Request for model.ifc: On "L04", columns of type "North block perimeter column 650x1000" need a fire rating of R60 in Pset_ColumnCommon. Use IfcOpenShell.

First a look at what the model holds.

```python
import ifcopenshell
import ifcopenshell.util.element

model = ifcopenshell.open("model.ifc")
print(model.schema)
storey = next(s for s in model.by_type("IfcBuildingStorey") if s.Name == "L04")
columns = [e for e in ifcopenshell.util.element.get_decomposition(storey) if e.is_a("IfcColumn")]
seen = {}
for e in columns:
    element_type = ifcopenshell.util.element.get_type(e)
    key = (element_type.Name if element_type != e and element_type else None, ifcopenshell.util.element.get_pset(e, "Pset_ColumnCommon", "FireRating"))
    seen[key] = seen.get(key, 0) + 1
for (name, value), count in sorted(seen.items(), key=str):
    print(count, "x", name, "|", value)
```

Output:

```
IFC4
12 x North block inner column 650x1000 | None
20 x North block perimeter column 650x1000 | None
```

```python
import ifcopenshell
import ifcopenshell.api.pset
import ifcopenshell.util.element

model = ifcopenshell.open("model.ifc")

storey = next(s for s in model.by_type("IfcBuildingStorey") if s.Name == "L04")
columns = [e for e in ifcopenshell.util.element.get_decomposition(storey) if e.is_a("IfcColumn")]

count = 0
for e in columns:
    element_type = ifcopenshell.util.element.get_type(e)
    if element_type in (None, e) or element_type.Name != "North block perimeter column 650x1000":
        continue
    # add_pset returns the element's existing set when there is one.
    pset = ifcopenshell.api.pset.add_pset(model, product=e, name="Pset_ColumnCommon")
    ifcopenshell.api.pset.edit_pset(model, pset=pset, properties={"FireRating": "R60"})
    count += 1

print(count, "columns updated")

model.write("model_v2.ifc")
```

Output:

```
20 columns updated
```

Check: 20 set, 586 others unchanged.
